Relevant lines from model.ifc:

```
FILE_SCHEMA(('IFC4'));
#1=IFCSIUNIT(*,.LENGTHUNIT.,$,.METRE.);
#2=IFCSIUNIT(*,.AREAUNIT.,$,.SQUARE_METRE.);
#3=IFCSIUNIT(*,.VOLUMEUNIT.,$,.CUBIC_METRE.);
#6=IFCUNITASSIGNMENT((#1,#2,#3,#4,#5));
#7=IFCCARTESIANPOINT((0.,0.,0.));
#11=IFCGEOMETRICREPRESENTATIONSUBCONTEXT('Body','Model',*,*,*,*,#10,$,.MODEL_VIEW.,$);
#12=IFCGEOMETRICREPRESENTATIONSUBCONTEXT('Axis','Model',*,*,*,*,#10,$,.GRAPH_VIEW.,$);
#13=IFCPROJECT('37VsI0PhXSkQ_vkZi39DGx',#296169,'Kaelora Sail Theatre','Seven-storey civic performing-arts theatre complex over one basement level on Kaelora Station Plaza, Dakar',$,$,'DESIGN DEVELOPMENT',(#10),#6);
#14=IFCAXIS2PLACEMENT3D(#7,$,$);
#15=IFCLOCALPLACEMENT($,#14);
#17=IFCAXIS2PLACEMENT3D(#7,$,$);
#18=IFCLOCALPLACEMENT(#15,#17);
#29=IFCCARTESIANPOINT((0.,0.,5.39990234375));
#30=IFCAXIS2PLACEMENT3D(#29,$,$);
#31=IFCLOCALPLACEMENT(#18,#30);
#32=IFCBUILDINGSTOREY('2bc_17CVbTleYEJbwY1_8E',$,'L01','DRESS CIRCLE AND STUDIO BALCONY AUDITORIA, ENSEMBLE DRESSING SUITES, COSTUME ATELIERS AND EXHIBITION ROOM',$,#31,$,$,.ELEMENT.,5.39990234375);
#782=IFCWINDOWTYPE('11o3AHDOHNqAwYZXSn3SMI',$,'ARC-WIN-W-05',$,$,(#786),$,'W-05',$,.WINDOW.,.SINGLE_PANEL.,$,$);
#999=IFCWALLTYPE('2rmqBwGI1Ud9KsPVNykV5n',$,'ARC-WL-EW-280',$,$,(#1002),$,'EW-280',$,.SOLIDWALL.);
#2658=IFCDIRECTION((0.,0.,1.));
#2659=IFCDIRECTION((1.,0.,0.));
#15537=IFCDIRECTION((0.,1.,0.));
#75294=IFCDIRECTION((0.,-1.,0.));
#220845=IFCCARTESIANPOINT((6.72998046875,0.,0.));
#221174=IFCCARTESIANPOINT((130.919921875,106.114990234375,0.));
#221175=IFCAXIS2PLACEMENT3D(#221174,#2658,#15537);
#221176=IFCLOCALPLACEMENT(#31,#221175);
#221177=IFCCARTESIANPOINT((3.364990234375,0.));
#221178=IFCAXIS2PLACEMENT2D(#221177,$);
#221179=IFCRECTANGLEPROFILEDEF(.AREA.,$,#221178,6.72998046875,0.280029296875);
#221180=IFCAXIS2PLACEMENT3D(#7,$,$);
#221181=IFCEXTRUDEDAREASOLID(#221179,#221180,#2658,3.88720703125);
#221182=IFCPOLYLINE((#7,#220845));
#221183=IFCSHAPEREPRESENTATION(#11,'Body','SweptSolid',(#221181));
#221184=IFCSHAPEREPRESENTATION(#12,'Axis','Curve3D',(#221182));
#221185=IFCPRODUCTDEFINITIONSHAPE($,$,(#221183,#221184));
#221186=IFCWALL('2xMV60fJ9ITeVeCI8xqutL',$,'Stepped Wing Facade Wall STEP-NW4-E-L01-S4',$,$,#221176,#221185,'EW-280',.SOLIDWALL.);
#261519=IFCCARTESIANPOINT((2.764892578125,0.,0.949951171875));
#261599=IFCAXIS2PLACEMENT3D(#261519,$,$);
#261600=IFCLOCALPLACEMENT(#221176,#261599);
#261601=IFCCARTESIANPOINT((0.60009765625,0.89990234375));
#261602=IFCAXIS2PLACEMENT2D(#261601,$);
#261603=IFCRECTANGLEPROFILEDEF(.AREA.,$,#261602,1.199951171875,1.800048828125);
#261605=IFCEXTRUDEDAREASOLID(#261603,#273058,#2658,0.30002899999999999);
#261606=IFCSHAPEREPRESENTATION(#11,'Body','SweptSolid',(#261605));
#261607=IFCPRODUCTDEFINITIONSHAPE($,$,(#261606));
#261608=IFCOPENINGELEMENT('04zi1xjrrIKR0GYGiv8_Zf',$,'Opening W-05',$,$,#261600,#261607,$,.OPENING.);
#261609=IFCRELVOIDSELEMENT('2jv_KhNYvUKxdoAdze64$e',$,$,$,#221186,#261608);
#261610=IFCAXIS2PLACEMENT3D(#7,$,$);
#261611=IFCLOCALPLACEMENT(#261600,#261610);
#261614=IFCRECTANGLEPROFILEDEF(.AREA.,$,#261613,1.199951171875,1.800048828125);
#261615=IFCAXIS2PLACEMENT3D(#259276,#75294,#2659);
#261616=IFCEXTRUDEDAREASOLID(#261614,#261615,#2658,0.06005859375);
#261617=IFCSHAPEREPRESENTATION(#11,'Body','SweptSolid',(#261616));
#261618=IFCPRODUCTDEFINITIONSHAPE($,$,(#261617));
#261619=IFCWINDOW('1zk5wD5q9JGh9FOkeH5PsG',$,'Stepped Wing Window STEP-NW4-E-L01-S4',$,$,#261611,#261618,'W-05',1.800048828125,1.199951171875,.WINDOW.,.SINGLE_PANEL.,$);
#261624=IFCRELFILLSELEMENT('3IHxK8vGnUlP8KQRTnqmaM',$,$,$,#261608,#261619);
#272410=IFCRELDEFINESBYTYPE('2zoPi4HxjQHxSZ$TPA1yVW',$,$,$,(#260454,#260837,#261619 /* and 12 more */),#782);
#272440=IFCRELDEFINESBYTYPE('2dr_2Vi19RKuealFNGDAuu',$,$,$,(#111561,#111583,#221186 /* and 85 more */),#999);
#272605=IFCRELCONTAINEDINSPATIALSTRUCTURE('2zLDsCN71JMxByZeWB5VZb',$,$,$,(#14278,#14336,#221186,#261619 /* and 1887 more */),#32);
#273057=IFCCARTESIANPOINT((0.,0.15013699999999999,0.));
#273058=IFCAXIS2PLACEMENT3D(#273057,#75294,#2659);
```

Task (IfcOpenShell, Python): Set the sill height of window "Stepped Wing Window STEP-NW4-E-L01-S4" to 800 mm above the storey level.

```python
import numpy as np
import ifcopenshell
import ifcopenshell.api.geometry
import ifcopenshell.geom
import ifcopenshell.util.element
import ifcopenshell.util.placement
import ifcopenshell.util.shape
import ifcopenshell.util.unit

model = ifcopenshell.open("model.ifc")
unit_scale = ifcopenshell.util.unit.calculate_unit_scale(model)

window = model.by_guid("1zk5wD5q9JGh9FOkeH5PsG")
opening = window.FillsVoids[0].RelatingOpeningElement
storey = ifcopenshell.util.element.get_container(window, ifc_class="IfcBuildingStorey")
level = ifcopenshell.util.placement.get_local_placement(storey.ObjectPlacement)[2, 3]

# The opening's origin need not be at the sill, so measure its lowest point.
shape = ifcopenshell.geom.create_shape(ifcopenshell.geom.settings(), opening)
bottom = ifcopenshell.util.shape.get_shape_bottom_elevation(shape, shape.geometry) / unit_scale
dz = level + 0.8 - bottom

shift = np.array([0.0, 0.0, dz])
# The window is placed relative to its opening, so it follows when the opening moves.
matrix = ifcopenshell.util.placement.get_local_placement(opening.ObjectPlacement)
matrix[:3, 3] += shift
ifcopenshell.api.geometry.edit_object_placement(
    model, product=opening, matrix=matrix, is_si=False, should_transform_children=True
)

print(f"moved by {dz * unit_scale:+.3f} m")

model.write("model-out.ifc")
```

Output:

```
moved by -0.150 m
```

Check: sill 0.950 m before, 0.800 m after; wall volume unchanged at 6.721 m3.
